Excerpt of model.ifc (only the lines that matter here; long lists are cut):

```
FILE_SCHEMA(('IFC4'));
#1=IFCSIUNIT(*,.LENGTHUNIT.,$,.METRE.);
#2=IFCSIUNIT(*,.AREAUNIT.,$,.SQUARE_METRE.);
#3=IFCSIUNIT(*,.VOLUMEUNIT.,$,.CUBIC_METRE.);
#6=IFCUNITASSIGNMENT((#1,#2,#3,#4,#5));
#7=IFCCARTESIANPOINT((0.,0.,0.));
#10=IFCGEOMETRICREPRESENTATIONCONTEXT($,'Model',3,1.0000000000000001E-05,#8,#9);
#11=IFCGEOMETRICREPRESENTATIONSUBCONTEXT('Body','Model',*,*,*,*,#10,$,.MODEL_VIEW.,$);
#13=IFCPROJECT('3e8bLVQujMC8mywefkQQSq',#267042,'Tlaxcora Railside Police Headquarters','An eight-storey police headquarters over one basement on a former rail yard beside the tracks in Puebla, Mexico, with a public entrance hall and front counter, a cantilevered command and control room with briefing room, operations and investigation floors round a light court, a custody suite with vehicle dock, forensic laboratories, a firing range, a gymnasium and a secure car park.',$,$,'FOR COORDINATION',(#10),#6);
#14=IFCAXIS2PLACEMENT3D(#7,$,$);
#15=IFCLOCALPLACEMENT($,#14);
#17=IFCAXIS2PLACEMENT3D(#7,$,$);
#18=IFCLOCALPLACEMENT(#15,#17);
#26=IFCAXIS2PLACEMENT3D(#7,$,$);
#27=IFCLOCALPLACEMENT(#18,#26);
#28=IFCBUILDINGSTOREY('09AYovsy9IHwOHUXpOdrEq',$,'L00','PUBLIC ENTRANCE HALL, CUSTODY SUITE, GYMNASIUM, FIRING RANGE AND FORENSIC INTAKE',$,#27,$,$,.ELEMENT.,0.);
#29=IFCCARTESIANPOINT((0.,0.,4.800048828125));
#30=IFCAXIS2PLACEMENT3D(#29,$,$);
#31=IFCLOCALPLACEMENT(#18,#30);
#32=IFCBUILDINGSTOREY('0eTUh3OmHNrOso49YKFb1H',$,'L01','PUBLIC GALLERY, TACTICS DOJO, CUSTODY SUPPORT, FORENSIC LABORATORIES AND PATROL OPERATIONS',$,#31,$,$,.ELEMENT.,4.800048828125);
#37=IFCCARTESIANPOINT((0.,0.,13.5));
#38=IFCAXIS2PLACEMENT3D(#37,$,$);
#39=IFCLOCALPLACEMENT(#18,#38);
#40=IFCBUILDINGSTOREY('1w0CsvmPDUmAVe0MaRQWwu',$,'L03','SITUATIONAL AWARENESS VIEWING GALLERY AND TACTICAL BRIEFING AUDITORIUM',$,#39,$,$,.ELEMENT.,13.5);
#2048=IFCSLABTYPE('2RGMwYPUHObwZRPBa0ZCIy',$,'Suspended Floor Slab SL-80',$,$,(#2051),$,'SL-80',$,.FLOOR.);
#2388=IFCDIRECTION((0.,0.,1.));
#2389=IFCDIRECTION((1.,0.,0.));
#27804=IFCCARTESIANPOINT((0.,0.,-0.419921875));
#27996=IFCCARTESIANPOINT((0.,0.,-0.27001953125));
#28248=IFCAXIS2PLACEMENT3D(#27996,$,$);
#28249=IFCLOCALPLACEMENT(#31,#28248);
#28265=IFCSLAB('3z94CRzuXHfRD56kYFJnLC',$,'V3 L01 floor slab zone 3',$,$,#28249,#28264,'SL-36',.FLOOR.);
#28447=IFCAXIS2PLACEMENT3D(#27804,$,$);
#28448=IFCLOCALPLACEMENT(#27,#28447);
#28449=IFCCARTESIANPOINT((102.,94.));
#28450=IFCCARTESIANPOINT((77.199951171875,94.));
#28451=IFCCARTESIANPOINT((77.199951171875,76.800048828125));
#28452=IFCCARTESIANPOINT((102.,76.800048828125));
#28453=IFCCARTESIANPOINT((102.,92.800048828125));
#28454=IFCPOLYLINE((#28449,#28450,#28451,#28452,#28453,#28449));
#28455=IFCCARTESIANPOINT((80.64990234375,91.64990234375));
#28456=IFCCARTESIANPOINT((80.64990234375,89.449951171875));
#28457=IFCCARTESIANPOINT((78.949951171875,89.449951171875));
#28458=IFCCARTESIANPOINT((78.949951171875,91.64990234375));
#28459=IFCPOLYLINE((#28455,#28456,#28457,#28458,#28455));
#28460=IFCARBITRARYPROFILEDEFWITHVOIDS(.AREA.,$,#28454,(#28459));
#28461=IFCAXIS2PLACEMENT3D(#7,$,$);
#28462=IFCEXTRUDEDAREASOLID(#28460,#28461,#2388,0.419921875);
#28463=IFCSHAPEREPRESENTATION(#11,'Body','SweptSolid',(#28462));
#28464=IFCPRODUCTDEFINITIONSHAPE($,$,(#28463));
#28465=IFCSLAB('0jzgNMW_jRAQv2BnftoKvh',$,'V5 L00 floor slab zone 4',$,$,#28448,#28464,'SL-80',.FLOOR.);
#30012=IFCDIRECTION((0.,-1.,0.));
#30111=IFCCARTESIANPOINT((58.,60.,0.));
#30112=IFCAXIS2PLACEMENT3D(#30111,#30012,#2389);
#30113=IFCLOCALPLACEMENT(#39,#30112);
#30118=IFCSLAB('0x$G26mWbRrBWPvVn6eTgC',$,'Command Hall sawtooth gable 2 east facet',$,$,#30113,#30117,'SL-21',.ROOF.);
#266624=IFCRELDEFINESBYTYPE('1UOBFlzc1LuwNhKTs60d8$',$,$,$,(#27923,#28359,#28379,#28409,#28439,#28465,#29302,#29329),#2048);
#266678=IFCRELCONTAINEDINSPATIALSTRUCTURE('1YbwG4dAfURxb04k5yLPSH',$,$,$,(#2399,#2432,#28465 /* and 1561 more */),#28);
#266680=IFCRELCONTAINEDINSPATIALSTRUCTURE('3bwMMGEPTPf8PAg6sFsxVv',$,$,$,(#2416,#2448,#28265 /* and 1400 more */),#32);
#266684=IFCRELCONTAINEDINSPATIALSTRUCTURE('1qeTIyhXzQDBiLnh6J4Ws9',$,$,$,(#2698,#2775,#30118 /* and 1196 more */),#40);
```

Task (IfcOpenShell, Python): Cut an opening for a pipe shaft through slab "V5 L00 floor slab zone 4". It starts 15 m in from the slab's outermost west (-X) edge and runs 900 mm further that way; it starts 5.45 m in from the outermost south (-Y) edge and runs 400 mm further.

```python
import numpy as np
import ifcopenshell
import ifcopenshell.api.feature
import ifcopenshell.api.geometry
import ifcopenshell.api.root
import ifcopenshell.geom
import ifcopenshell.util.placement
import ifcopenshell.util.representation
import ifcopenshell.util.shape
import ifcopenshell.util.unit

model = ifcopenshell.open("model.ifc")
unit_scale = ifcopenshell.util.unit.calculate_unit_scale(model)
settings = ifcopenshell.geom.settings()


def volume(element):
    """Net volume in cubic metres, openings subtracted."""
    shape = ifcopenshell.geom.create_shape(settings, element)
    return ifcopenshell.util.shape.get_volume(shape.geometry)


slab = model.by_guid("0jzgNMW_jRAQv2BnftoKvh")
before = volume(slab)

# Extent in the slab's own axes, in metres. The edges named are its -X and -Y sides.
slab_shape = ifcopenshell.geom.create_shape(settings, slab)
vertices = ifcopenshell.util.shape.get_vertices(slab_shape.geometry)
x_min, y_min, bottom = vertices.min(axis=0)
top = vertices[:, 2].max()

opening = ifcopenshell.api.root.create_entity(model, ifc_class="IfcOpeningElement", name="Pipe shaft opening", predefined_type="OPENING")
context = ifcopenshell.util.representation.get_context(model, "Model", "Body", "MODEL_VIEW")
width, depth = 0.9, 0.4
outline = [(0.0, 0.0), (width, 0.0), (width, depth), (0.0, depth), (0.0, 0.0)]
# Overshoot both faces by 50 mm so the cut is clean.
shape = ifcopenshell.api.geometry.add_slab_representation(
    model, context=context, depth=top - bottom + 0.1, polyline=outline
)
ifcopenshell.api.geometry.assign_representation(model, product=opening, representation=shape)

matrix = ifcopenshell.util.placement.get_local_placement(slab.ObjectPlacement)
matrix[:, 3] = matrix @ np.append(np.array([x_min + 15, y_min + 5.45, bottom - 0.05]) / unit_scale, 1.0)
ifcopenshell.api.geometry.edit_object_placement(model, product=opening, matrix=matrix, is_si=False)
ifcopenshell.api.feature.add_feature(model, feature=opening, element=slab)

after = volume(slab)

print(f"slab volume {before:.3f} -> {after:.3f} m3")

model.write("model_updated.ifc")
```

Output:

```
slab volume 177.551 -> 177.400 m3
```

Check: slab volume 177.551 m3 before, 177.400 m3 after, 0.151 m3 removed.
